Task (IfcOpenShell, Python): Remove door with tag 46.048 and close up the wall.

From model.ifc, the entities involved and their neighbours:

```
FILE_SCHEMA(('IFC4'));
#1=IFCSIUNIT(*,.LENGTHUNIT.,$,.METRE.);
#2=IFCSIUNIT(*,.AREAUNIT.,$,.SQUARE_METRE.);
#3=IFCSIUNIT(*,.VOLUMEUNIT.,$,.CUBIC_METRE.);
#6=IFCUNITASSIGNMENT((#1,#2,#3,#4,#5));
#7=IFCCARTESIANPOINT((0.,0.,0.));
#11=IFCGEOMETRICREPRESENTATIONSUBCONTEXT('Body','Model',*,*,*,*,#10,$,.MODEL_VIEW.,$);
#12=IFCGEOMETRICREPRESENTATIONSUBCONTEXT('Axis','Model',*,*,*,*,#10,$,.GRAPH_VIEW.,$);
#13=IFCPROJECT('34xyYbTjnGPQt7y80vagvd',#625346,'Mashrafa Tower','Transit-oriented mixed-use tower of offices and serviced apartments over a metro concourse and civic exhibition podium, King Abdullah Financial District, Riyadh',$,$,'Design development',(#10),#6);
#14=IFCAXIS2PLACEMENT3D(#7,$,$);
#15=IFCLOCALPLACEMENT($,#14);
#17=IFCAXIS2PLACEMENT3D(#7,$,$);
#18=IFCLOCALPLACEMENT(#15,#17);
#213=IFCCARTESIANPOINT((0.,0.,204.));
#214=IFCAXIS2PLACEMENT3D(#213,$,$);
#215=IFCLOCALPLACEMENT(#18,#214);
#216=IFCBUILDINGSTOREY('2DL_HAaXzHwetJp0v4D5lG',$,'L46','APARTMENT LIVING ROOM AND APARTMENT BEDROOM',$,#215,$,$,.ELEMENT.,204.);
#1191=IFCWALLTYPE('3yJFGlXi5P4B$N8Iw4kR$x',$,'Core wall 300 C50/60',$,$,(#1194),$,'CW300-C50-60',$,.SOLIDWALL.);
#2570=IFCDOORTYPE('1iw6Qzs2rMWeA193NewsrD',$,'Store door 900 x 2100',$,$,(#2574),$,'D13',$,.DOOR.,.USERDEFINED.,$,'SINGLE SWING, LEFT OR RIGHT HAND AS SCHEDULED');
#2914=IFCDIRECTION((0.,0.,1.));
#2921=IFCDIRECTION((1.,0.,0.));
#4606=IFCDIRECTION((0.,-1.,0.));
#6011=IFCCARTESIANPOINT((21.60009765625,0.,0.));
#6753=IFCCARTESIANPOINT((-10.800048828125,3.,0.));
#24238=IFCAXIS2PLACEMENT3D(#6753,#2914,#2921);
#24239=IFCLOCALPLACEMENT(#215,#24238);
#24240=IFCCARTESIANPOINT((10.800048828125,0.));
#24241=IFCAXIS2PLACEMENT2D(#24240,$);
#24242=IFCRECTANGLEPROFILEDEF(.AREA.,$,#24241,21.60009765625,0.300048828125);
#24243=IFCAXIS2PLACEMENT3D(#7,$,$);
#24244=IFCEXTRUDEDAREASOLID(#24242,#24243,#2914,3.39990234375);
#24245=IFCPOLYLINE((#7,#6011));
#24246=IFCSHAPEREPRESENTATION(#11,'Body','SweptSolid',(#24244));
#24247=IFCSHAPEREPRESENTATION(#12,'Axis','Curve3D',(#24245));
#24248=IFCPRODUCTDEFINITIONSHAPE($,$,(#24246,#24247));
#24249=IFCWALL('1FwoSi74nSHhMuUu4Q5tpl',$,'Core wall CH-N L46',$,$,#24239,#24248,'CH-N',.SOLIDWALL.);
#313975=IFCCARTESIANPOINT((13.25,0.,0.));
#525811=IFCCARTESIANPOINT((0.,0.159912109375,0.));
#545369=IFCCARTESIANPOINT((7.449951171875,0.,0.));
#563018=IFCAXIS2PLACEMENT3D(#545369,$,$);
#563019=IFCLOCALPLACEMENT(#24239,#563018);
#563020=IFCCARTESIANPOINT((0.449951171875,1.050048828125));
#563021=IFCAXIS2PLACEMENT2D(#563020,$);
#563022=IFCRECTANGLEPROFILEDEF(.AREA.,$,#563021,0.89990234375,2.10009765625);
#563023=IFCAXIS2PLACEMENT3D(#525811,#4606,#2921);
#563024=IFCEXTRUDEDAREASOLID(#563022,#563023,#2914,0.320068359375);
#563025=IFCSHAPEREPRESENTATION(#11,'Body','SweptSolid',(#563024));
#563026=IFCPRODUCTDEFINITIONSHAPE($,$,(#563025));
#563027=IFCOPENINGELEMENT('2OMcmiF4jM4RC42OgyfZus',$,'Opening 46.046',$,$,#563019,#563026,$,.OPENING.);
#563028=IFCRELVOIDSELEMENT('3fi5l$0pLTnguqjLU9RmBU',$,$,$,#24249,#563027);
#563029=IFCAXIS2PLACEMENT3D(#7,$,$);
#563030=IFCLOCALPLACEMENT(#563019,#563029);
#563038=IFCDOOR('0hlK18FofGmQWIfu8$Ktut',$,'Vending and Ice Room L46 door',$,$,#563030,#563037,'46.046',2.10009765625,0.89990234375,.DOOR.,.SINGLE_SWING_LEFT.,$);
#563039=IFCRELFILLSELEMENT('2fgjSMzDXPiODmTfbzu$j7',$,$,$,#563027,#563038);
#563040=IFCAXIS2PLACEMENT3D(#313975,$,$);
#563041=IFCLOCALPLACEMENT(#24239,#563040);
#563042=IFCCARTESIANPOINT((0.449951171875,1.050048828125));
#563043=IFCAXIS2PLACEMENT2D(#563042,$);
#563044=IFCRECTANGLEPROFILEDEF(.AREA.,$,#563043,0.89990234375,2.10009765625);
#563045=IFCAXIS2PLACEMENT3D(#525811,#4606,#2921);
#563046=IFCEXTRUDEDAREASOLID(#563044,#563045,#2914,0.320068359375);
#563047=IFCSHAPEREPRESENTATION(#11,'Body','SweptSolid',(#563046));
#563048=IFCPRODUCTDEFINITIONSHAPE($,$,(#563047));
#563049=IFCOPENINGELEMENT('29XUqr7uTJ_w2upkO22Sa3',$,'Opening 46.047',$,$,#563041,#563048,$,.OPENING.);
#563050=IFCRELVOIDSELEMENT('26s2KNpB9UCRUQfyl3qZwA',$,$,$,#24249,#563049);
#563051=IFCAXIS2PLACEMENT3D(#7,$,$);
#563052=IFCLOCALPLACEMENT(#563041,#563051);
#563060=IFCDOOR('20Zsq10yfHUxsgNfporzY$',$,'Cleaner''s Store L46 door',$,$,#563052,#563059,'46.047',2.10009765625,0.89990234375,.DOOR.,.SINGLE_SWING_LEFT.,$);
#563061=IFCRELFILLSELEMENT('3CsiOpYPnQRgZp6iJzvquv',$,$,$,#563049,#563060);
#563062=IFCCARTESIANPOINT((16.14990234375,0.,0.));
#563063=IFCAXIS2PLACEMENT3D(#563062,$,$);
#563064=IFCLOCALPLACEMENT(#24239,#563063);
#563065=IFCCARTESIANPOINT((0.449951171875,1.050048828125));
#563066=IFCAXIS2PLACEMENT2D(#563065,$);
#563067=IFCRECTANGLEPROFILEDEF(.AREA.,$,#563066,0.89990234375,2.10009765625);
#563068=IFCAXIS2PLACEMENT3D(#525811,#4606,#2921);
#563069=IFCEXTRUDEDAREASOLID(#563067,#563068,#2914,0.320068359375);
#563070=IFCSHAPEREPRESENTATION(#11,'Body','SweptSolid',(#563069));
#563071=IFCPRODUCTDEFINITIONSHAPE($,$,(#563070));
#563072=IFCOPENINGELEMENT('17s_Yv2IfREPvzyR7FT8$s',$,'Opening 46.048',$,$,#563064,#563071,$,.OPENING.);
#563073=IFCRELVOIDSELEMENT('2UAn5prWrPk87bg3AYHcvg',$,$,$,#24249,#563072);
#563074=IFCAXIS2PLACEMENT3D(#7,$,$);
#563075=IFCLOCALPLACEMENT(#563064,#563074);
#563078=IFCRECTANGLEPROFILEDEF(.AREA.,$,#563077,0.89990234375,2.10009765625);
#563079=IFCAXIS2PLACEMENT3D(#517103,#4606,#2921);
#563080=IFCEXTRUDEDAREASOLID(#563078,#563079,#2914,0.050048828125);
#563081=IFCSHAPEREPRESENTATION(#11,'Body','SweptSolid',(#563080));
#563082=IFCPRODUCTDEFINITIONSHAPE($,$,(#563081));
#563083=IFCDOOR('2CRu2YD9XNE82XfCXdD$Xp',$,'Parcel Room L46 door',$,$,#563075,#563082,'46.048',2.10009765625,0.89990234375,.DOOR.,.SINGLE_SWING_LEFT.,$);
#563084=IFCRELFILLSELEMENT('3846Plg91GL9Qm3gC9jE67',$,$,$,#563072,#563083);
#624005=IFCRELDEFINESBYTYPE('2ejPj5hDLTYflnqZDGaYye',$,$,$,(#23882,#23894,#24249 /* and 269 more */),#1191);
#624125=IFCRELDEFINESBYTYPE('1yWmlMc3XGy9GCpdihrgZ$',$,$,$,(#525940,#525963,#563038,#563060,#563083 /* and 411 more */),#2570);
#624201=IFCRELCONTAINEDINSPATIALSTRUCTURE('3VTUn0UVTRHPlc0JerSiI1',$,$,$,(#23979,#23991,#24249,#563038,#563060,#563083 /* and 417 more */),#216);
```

```python
import ifcopenshell
import ifcopenshell.api.feature
import ifcopenshell.api.root
import ifcopenshell.geom
import ifcopenshell.util.shape

model = ifcopenshell.open("model.ifc")
settings = ifcopenshell.geom.settings()


def volume(element):
    """Net volume in cubic metres, openings subtracted."""
    shape = ifcopenshell.geom.create_shape(settings, element)
    return ifcopenshell.util.shape.get_volume(shape.geometry)


door = model.by_guid("2CRu2YD9XNE82XfCXdD$Xp")
opening = door.FillsVoids[0].RelatingOpeningElement
wall = opening.VoidsElements[0].RelatingBuildingElement
before = volume(wall)

ifcopenshell.api.root.remove_product(model, product=door)
ifcopenshell.api.feature.remove_feature(model, feature=opening)

after = volume(wall)

print(f"wall volume {before:.3f} -> {after:.3f} m3")

model.write("model_v2.ifc")
```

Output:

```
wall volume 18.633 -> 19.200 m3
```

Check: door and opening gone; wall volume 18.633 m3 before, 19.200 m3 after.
